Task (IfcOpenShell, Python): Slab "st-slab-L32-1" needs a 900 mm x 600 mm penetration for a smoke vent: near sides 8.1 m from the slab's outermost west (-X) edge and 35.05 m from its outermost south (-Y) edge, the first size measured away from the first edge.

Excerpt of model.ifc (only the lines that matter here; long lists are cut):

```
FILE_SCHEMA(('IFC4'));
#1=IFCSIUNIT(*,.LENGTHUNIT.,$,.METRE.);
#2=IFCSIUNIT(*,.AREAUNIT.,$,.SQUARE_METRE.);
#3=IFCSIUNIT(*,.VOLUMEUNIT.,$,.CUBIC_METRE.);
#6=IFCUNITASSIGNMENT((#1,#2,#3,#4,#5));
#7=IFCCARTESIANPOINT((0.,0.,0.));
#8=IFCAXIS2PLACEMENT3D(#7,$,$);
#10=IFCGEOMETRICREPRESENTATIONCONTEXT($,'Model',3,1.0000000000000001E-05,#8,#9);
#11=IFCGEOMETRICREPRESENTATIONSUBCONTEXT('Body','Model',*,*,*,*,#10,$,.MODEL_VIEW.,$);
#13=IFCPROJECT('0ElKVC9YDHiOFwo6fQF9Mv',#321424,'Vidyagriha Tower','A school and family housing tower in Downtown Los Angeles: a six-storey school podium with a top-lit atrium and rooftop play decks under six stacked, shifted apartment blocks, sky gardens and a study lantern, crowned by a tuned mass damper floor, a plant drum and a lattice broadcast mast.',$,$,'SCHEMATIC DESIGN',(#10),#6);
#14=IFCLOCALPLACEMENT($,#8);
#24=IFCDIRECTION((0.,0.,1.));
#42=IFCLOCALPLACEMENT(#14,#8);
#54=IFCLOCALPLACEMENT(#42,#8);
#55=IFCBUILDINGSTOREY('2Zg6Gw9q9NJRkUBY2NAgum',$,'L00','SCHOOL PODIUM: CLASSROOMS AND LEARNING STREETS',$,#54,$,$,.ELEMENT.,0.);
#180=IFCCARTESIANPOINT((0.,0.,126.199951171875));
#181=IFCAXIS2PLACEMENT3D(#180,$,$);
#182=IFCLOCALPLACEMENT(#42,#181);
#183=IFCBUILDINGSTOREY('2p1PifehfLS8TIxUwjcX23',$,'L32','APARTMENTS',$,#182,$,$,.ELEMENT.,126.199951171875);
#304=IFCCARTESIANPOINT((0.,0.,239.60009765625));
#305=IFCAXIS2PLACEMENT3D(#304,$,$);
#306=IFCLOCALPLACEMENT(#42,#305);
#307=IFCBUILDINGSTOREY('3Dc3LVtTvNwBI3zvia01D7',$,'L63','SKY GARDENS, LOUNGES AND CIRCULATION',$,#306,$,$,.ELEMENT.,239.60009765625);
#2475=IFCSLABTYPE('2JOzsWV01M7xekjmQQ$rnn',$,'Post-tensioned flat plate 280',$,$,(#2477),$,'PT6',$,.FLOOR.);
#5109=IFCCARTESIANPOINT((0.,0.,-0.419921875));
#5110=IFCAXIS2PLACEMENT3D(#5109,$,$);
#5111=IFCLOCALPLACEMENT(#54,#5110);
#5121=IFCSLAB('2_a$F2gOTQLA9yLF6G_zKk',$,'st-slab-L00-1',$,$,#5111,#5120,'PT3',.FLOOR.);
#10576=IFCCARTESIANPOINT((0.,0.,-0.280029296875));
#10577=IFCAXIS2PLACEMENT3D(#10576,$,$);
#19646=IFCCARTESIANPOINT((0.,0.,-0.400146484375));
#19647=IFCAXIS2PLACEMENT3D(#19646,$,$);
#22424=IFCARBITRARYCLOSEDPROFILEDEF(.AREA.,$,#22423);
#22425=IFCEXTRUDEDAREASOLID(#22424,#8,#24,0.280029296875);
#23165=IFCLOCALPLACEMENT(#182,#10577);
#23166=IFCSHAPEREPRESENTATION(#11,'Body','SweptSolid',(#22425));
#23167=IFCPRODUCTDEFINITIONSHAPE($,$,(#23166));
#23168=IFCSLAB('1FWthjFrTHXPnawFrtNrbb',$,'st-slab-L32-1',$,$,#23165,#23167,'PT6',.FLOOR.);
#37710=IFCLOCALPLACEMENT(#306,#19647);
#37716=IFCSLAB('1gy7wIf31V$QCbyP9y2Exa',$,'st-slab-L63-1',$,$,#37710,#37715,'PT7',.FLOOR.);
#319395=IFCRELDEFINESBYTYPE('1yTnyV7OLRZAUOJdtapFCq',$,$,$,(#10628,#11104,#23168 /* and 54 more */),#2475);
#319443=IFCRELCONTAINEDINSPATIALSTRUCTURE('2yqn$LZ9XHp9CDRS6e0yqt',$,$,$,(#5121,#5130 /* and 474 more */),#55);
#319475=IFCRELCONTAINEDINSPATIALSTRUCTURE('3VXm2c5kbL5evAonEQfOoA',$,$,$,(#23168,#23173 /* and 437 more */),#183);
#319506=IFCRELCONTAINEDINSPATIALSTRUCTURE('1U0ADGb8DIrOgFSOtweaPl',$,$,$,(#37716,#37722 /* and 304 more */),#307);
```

```python
import numpy as np
import ifcopenshell
import ifcopenshell.api.feature
import ifcopenshell.api.geometry
import ifcopenshell.api.root
import ifcopenshell.geom
import ifcopenshell.util.placement
import ifcopenshell.util.representation
import ifcopenshell.util.shape
import ifcopenshell.util.unit

model = ifcopenshell.open("model.ifc")
unit_scale = ifcopenshell.util.unit.calculate_unit_scale(model)
settings = ifcopenshell.geom.settings()


def volume(element):
    """Net volume in cubic metres, openings subtracted."""
    shape = ifcopenshell.geom.create_shape(settings, element)
    return ifcopenshell.util.shape.get_volume(shape.geometry)


slab = model.by_guid("1FWthjFrTHXPnawFrtNrbb")
before = volume(slab)

# Extent in the slab's own axes, in metres. The edges named are its -X and -Y sides.
slab_shape = ifcopenshell.geom.create_shape(settings, slab)
vertices = ifcopenshell.util.shape.get_vertices(slab_shape.geometry)
x_min, y_min, bottom = vertices.min(axis=0)
top = vertices[:, 2].max()

opening = ifcopenshell.api.root.create_entity(model, ifc_class="IfcOpeningElement", name="Smoke vent opening", predefined_type="OPENING")
context = ifcopenshell.util.representation.get_context(model, "Model", "Body", "MODEL_VIEW")
width, depth = 0.9, 0.6
outline = [(0.0, 0.0), (width, 0.0), (width, depth), (0.0, depth), (0.0, 0.0)]
# Overshoot both faces by 50 mm so the cut is clean.
shape = ifcopenshell.api.geometry.add_slab_representation(
    model, context=context, depth=top - bottom + 0.1, polyline=outline
)
ifcopenshell.api.geometry.assign_representation(model, product=opening, representation=shape)

matrix = ifcopenshell.util.placement.get_local_placement(slab.ObjectPlacement)
matrix[:, 3] = matrix @ np.append(np.array([x_min + 8.1, y_min + 35.05, bottom - 0.05]) / unit_scale, 1.0)
ifcopenshell.api.geometry.edit_object_placement(model, product=opening, matrix=matrix, is_si=False)
ifcopenshell.api.feature.add_feature(model, feature=opening, element=slab)

after = volume(slab)

print(f"slab volume {before:.3f} -> {after:.3f} m3")

model.write("model_v2.ifc")
```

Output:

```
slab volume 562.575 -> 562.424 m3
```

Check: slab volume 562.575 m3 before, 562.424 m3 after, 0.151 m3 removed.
